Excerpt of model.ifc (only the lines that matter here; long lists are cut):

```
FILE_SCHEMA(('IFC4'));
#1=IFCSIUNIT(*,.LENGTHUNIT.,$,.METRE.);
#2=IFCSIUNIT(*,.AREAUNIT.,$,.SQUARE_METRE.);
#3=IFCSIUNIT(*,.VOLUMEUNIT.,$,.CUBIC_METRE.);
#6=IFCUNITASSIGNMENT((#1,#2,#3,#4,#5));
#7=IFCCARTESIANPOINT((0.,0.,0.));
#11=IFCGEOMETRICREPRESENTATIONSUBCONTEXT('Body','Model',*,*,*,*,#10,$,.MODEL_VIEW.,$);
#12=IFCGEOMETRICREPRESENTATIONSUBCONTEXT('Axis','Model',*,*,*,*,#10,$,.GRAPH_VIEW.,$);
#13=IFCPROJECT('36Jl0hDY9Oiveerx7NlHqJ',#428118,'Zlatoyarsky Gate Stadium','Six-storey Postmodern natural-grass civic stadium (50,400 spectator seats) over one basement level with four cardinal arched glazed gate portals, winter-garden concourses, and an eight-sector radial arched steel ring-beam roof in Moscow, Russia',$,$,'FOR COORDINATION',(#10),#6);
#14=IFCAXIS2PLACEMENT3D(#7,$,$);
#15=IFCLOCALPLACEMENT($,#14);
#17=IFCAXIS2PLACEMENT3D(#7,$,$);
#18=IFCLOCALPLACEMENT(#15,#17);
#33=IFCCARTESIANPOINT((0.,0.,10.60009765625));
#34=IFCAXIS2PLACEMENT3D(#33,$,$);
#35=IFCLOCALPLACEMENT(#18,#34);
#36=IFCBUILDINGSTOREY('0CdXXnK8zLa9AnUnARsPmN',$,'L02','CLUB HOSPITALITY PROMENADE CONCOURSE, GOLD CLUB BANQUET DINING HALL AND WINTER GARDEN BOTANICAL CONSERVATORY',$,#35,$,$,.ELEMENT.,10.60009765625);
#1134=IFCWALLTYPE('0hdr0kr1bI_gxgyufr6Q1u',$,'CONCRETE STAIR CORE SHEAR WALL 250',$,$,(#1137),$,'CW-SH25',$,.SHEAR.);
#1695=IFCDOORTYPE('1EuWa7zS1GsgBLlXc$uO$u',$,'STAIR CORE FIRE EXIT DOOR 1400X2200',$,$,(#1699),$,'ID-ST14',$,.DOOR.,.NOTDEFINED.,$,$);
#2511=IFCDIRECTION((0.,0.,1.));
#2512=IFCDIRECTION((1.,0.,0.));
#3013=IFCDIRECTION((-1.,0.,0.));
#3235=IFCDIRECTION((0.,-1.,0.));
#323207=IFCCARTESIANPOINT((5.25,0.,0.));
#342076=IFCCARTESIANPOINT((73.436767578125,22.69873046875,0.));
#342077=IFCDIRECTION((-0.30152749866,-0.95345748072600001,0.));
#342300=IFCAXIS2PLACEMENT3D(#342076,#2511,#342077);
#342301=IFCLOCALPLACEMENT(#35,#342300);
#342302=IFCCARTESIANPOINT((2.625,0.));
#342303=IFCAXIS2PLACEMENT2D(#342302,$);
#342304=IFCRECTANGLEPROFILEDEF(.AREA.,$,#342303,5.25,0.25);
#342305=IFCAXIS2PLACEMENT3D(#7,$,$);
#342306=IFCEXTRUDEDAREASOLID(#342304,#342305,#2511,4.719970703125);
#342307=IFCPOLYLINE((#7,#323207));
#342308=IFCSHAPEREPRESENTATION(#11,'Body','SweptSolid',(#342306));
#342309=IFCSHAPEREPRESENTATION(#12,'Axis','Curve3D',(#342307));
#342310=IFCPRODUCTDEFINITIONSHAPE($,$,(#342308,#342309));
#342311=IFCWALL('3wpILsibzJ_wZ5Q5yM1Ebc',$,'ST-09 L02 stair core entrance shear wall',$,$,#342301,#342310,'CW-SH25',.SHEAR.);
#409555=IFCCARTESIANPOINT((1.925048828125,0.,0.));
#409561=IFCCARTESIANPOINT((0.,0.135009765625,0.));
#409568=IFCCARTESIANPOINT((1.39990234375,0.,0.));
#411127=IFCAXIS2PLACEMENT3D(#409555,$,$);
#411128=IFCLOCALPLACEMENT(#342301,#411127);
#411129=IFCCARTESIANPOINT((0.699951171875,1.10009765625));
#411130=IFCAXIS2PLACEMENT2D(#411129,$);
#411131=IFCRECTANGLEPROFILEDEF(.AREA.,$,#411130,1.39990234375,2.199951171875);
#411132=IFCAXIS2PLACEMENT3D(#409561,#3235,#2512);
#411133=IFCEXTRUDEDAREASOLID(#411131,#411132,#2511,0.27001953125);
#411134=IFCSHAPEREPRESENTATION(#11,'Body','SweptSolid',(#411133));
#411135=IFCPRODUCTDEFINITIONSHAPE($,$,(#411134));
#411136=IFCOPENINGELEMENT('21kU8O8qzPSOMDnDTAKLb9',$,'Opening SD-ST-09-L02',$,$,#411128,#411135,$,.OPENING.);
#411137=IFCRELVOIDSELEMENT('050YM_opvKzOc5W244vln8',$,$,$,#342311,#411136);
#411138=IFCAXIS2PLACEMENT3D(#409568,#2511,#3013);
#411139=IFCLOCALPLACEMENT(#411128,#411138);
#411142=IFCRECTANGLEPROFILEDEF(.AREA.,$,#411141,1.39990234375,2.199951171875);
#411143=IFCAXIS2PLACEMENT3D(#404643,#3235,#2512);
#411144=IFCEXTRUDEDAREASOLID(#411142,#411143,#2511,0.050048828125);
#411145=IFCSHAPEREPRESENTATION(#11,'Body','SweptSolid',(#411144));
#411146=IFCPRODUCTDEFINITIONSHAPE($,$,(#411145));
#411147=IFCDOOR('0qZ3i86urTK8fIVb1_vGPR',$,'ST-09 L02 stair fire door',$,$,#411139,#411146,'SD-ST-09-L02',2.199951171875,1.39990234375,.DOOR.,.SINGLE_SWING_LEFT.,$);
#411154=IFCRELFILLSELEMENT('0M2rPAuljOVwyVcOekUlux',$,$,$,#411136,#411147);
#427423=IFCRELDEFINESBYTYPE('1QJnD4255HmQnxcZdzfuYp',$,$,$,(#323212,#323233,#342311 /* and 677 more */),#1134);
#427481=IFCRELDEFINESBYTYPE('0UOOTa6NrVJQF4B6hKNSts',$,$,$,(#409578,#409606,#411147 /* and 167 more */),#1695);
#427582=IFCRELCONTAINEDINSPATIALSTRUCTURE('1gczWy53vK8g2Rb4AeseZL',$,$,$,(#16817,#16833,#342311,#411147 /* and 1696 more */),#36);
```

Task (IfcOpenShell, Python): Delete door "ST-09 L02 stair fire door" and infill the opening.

```python
import ifcopenshell
import ifcopenshell.api.feature
import ifcopenshell.api.root
import ifcopenshell.geom
import ifcopenshell.util.shape

model = ifcopenshell.open("model.ifc")
settings = ifcopenshell.geom.settings()


def volume(element):
    """Net volume in cubic metres, openings subtracted."""
    shape = ifcopenshell.geom.create_shape(settings, element)
    return ifcopenshell.util.shape.get_volume(shape.geometry)


door = model.by_guid("0qZ3i86urTK8fIVb1_vGPR")
opening = door.FillsVoids[0].RelatingOpeningElement
wall = opening.VoidsElements[0].RelatingBuildingElement
before = volume(wall)

ifcopenshell.api.root.remove_product(model, product=door)
ifcopenshell.api.feature.remove_feature(model, feature=opening)

after = volume(wall)

print(f"wall volume {before:.3f} -> {after:.3f} m3")

model.write("model_edited.ifc")
```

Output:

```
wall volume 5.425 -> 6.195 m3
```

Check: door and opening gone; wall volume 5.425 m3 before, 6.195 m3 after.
